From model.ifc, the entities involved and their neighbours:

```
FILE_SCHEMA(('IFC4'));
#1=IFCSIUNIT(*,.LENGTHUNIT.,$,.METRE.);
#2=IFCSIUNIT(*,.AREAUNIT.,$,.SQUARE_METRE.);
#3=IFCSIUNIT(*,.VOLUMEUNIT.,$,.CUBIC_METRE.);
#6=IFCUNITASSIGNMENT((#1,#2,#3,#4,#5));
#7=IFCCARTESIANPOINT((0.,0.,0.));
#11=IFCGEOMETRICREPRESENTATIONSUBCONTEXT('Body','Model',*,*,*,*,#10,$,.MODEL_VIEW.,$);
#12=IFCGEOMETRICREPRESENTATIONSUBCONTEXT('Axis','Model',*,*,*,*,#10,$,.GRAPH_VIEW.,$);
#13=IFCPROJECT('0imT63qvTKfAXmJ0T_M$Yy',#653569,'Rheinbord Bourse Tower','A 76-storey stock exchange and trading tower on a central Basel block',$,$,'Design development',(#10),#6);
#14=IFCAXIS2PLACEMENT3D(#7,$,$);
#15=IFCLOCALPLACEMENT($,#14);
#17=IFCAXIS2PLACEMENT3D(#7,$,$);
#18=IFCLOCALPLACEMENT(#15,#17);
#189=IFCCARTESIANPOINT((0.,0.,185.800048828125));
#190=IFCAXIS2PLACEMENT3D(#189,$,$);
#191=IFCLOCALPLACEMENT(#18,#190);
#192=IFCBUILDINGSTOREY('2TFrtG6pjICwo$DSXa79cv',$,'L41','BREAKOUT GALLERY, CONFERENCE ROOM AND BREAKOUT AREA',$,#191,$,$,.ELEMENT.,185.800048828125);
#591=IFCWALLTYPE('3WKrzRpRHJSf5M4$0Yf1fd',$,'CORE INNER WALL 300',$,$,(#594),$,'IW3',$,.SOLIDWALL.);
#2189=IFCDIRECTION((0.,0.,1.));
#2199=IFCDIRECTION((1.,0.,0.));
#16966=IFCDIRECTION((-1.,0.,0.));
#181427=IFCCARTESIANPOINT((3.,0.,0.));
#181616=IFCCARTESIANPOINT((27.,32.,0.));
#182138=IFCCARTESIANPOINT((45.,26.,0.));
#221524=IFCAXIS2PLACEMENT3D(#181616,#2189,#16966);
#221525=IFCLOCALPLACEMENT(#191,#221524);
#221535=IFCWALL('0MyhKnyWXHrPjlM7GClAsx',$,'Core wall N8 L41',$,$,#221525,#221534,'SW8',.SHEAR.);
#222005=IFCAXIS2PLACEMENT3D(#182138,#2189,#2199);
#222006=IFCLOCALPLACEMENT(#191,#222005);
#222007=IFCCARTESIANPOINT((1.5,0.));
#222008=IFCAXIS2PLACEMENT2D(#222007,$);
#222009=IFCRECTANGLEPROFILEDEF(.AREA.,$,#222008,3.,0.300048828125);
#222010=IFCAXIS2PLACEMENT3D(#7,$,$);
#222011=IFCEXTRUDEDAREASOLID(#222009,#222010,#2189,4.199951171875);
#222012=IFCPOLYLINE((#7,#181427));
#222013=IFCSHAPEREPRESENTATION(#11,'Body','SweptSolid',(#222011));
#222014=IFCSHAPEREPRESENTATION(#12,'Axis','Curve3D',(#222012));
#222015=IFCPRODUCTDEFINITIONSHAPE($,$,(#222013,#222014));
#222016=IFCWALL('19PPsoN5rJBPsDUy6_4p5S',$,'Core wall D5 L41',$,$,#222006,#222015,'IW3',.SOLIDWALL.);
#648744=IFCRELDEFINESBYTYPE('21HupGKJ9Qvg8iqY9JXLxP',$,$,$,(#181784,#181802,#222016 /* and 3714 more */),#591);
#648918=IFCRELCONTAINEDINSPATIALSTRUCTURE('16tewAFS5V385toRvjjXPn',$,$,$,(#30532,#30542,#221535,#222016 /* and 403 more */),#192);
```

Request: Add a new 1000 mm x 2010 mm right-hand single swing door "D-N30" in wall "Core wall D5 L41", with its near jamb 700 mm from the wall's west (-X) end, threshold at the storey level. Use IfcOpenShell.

```python
import numpy as np
import ifcopenshell
import ifcopenshell.api.feature
import ifcopenshell.api.geometry
import ifcopenshell.api.root
import ifcopenshell.api.spatial
import ifcopenshell.geom
import ifcopenshell.util.element
import ifcopenshell.util.placement
import ifcopenshell.util.representation
import ifcopenshell.util.shape
import ifcopenshell.util.unit

model = ifcopenshell.open("model.ifc")
unit_scale = ifcopenshell.util.unit.calculate_unit_scale(model)
settings = ifcopenshell.geom.settings()


def volume(element):
    """Net volume in cubic metres, openings subtracted."""
    shape = ifcopenshell.geom.create_shape(settings, element)
    return ifcopenshell.util.shape.get_volume(shape.geometry)


wall = model.by_guid("19PPsoN5rJBPsDUy6_4p5S")
storey = ifcopenshell.util.element.get_container(wall, ifc_class="IfcBuildingStorey")
context = ifcopenshell.util.representation.get_context(model, "Model", "Body", "MODEL_VIEW")
before = volume(wall)

width, height, from_end, sill = 1, 2.01, 0.7, 0.0  # metres

# The wall runs along its own X axis, and the end named is its -X end.
wall_shape = ifcopenshell.geom.create_shape(settings, wall)
x, y, z = ifcopenshell.util.shape.get_vertices(wall_shape.geometry).T
start = x.min() + from_end
face, thickness = float(y.min()), float(y.max() - y.min())
wall_matrix = ifcopenshell.util.placement.get_local_placement(wall.ObjectPlacement)
level = ifcopenshell.util.placement.get_local_placement(storey.ObjectPlacement)[2, 3]


def in_wall(x, y):
    """Placement at x, y metres in the wall's axes, at sill height."""
    matrix = wall_matrix.copy()
    matrix[:, 3] = wall_matrix @ np.array([x / unit_scale, y / unit_scale, 0.0, 1.0])
    matrix[2, 3] = level + sill / unit_scale
    return matrix


# Opening: a box that overshoots both wall faces by 50 mm.
opening = ifcopenshell.api.root.create_entity(model, ifc_class="IfcOpeningElement", predefined_type="OPENING")
box = ifcopenshell.api.geometry.add_wall_representation(
    model, context=context, length=width, height=height, thickness=thickness + 0.1
)
ifcopenshell.api.geometry.assign_representation(model, product=opening, representation=box)
ifcopenshell.api.geometry.edit_object_placement(model, product=opening, matrix=in_wall(start, face - 0.05), is_si=False)
ifcopenshell.api.feature.add_feature(model, feature=opening, element=wall)

door = ifcopenshell.api.root.create_entity(model, ifc_class="IfcDoor", name="D-N30", predefined_type="DOOR")
door.OverallWidth, door.OverallHeight = width / unit_scale, height / unit_scale
door.OperationType = "SINGLE_SWING_RIGHT"
body = ifcopenshell.api.geometry.add_door_representation(
    model,
    context=context,
    overall_width=door.OverallWidth,
    overall_height=door.OverallHeight,
    operation_type="SINGLE_SWING_RIGHT",
    lining_properties={"LiningDepth": thickness / unit_scale, "ThresholdDepth": thickness / unit_scale},
)
ifcopenshell.api.geometry.assign_representation(model, product=door, representation=body)
ifcopenshell.api.spatial.assign_container(model, products=[door], relating_structure=storey)
ifcopenshell.api.feature.add_filling(model, opening=opening, element=door)

# The lining spans the wall, so the door starts at the wall face.
ifcopenshell.api.geometry.edit_object_placement(model, product=door, matrix=in_wall(start, face), is_si=False)

after = volume(wall)

print(f"wall volume {before:.3f} -> {after:.3f} m3")

model.write("model_v2.ifc")
```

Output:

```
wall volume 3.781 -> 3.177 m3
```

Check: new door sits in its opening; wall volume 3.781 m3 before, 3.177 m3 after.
